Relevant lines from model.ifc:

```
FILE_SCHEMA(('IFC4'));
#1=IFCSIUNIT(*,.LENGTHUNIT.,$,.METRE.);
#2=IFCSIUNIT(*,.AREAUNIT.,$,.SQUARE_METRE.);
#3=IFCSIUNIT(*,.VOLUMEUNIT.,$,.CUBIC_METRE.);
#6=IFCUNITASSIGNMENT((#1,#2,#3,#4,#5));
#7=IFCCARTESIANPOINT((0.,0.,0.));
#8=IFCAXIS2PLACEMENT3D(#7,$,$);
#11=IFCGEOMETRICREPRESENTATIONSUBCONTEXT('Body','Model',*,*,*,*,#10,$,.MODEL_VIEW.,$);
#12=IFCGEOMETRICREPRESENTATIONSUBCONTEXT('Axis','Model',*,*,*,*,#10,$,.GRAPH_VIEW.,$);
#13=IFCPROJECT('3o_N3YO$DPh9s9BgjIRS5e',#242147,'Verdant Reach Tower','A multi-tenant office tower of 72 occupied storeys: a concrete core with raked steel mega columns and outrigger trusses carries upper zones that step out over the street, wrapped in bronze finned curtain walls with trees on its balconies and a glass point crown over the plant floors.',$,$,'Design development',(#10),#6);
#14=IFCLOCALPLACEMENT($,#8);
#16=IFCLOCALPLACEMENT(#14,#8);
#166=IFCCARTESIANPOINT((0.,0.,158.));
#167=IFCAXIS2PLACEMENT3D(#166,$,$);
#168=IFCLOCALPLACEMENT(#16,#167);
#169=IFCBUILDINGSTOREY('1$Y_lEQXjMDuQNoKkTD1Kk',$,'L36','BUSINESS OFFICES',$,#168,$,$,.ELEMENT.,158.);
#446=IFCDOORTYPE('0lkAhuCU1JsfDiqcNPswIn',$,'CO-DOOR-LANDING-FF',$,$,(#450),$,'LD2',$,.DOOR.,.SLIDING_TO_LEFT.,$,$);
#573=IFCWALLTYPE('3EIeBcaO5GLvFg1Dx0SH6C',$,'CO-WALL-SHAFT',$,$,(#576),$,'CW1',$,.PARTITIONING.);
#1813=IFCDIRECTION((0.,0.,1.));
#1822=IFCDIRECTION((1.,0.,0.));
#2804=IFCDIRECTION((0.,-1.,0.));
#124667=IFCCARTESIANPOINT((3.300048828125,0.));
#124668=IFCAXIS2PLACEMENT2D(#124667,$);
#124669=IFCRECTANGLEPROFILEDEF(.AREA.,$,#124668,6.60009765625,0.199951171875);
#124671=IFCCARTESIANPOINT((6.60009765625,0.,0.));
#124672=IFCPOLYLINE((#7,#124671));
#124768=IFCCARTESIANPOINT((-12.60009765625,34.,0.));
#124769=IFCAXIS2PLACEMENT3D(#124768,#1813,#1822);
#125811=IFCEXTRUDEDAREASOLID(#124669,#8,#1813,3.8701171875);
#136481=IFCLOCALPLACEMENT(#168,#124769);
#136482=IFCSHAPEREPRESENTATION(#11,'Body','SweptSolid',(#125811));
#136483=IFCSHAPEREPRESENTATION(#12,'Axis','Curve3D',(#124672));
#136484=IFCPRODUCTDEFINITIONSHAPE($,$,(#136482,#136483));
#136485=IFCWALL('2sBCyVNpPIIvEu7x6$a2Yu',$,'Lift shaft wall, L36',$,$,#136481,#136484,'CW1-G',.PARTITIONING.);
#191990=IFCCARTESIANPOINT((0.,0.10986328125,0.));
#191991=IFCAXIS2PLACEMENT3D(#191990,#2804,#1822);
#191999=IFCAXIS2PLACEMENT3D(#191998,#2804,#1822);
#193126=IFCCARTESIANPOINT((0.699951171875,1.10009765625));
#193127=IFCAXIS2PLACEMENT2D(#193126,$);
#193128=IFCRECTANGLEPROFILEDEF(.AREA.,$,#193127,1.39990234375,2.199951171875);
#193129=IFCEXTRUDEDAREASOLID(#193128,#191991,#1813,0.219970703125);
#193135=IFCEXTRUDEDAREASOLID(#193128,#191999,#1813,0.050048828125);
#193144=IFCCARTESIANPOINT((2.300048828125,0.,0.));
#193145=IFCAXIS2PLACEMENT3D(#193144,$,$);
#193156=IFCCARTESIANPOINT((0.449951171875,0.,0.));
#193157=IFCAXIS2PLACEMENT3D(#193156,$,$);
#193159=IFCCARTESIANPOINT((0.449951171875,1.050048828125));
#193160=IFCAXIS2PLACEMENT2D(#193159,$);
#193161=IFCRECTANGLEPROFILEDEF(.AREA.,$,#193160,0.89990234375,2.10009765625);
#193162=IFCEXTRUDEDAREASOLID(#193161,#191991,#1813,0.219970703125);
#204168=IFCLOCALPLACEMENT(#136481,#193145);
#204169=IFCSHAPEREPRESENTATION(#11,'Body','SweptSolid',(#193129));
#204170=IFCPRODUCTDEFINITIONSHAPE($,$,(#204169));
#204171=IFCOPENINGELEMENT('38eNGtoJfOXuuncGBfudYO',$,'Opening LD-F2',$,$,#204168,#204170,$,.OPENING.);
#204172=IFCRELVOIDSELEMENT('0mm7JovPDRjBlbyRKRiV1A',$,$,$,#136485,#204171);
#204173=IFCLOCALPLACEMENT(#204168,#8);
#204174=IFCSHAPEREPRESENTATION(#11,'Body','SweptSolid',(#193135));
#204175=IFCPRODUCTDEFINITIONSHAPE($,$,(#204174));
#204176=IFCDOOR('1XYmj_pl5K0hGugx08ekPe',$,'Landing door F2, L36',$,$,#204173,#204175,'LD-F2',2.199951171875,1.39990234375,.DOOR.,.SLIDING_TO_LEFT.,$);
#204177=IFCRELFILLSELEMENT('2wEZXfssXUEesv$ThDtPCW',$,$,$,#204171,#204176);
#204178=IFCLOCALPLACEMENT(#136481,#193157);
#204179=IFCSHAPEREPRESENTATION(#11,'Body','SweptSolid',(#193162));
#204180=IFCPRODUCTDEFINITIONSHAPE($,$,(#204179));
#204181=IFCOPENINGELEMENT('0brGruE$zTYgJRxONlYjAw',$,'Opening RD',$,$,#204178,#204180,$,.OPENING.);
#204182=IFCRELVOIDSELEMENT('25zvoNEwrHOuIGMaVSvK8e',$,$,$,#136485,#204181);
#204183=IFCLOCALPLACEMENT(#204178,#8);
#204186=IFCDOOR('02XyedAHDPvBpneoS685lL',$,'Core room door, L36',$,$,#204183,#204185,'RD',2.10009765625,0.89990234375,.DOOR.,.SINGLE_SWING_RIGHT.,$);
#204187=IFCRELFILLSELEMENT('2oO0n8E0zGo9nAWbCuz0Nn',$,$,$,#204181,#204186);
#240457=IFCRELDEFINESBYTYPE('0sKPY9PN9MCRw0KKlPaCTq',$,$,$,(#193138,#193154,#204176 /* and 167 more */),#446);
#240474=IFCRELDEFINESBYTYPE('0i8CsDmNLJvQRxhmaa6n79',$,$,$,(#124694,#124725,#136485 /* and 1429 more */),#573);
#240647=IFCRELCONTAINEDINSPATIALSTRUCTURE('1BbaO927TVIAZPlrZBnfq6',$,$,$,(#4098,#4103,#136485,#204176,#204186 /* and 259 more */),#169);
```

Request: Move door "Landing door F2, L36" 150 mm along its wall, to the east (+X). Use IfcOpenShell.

```python
import ifcopenshell
import ifcopenshell.api.geometry
import ifcopenshell.util.placement
import ifcopenshell.util.unit

model = ifcopenshell.open("model.ifc")
unit_scale = ifcopenshell.util.unit.calculate_unit_scale(model)

door = model.by_guid("1XYmj_pl5K0hGugx08ekPe")
opening = door.FillsVoids[0].RelatingOpeningElement
wall = opening.VoidsElements[0].RelatingBuildingElement

wall_matrix = ifcopenshell.util.placement.get_local_placement(wall.ObjectPlacement)
shift = wall_matrix[:3, 0] * 0.15 / unit_scale
before = ifcopenshell.util.placement.get_local_placement(door.ObjectPlacement)[:3, 3].copy()

# The door is placed relative to its opening, so it follows when the opening moves.
matrix = ifcopenshell.util.placement.get_local_placement(opening.ObjectPlacement)
matrix[:3, 3] += shift
ifcopenshell.api.geometry.edit_object_placement(
    model, product=opening, matrix=matrix, is_si=False, should_transform_children=True
)

after = ifcopenshell.util.placement.get_local_placement(door.ObjectPlacement)[:3, 3]
print("door moved by", (after - before).round(3) + 0.0)

model.write("model_v2.ifc")
```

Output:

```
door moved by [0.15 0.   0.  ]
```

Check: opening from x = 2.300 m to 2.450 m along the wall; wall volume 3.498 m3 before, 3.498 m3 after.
